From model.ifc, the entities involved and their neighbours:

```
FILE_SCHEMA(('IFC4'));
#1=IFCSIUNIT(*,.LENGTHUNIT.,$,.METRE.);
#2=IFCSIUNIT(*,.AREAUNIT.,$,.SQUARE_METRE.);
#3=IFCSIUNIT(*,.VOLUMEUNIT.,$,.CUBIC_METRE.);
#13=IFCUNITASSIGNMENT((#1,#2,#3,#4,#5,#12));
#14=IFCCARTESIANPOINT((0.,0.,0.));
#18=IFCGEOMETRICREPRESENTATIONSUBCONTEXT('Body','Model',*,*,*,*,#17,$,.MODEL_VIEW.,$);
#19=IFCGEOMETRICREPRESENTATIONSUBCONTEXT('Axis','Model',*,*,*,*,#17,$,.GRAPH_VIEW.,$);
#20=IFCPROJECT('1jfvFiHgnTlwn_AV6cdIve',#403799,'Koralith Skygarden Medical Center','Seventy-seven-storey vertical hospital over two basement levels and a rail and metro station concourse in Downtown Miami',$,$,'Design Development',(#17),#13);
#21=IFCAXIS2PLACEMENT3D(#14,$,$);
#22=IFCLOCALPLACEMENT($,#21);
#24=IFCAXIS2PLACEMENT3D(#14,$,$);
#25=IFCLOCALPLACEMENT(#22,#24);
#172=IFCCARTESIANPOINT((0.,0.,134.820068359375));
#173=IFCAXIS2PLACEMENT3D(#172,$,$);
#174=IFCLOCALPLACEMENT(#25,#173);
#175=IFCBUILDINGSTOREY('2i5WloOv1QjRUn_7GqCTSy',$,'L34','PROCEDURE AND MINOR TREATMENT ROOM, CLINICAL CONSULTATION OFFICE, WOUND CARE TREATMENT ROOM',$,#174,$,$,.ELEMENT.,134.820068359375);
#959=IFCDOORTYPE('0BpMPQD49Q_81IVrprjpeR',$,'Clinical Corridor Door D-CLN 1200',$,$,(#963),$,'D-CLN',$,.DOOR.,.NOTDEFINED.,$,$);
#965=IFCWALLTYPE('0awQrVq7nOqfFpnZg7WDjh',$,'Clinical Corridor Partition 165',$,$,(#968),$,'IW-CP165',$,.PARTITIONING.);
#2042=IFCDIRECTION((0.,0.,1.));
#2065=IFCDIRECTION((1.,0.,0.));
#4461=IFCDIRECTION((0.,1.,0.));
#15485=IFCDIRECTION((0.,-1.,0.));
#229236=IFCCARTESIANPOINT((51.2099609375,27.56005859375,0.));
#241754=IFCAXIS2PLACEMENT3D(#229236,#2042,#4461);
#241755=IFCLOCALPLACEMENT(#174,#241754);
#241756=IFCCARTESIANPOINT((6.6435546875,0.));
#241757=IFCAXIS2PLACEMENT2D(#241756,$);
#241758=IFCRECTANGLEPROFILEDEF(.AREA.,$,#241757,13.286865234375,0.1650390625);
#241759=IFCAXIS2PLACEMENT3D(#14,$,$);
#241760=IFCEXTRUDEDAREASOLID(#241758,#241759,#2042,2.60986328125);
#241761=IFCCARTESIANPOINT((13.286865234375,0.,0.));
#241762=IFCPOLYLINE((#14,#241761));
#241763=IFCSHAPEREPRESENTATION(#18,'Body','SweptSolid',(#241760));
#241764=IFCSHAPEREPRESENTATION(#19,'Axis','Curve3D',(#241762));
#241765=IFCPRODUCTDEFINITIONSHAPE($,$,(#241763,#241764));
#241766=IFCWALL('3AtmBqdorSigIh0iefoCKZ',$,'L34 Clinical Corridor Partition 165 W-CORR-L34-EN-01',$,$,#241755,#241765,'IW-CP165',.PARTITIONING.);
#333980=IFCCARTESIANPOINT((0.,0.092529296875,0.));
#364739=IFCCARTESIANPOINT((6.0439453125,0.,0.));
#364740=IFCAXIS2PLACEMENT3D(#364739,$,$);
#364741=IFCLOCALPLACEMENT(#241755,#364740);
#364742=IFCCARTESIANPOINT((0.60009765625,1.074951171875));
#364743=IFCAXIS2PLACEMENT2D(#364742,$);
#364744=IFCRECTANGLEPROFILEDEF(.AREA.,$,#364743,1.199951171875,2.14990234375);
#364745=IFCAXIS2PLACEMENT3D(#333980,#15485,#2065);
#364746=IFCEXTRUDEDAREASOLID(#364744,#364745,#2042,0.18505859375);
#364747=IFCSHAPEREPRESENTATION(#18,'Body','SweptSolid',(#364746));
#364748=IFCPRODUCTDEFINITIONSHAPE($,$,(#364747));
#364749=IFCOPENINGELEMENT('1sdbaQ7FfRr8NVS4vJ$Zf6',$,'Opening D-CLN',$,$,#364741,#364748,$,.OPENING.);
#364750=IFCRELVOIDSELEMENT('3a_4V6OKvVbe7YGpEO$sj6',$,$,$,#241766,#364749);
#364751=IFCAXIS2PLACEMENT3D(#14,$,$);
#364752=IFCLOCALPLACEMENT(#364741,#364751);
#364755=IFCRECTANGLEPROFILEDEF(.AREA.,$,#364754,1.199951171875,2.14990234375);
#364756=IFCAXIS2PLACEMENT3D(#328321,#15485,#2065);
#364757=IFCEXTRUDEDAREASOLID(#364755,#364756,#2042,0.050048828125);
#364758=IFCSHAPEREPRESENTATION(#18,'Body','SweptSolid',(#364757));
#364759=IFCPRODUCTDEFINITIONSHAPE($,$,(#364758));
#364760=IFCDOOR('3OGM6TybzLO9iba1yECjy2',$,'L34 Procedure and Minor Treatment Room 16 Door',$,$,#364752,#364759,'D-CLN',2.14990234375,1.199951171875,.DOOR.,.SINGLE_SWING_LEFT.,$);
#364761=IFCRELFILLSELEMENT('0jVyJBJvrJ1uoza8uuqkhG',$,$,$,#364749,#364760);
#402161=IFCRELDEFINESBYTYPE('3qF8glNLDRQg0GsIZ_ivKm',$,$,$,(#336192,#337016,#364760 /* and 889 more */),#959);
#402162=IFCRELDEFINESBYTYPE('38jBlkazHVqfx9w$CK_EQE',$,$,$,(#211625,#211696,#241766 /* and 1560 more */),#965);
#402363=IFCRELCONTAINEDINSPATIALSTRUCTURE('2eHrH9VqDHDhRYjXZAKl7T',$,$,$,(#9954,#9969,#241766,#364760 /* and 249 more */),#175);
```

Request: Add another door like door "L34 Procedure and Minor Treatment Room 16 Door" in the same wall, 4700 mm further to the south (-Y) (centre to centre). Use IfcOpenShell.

```python
import ifcopenshell
import ifcopenshell.api.feature
import ifcopenshell.api.geometry
import ifcopenshell.api.root
import ifcopenshell.geom
import ifcopenshell.util.element
import ifcopenshell.util.placement
import ifcopenshell.util.shape
import ifcopenshell.util.unit

model = ifcopenshell.open("model.ifc")
unit_scale = ifcopenshell.util.unit.calculate_unit_scale(model)
settings = ifcopenshell.geom.settings()


def volume(element):
    """Net volume in cubic metres, openings subtracted."""
    shape = ifcopenshell.geom.create_shape(settings, element)
    return ifcopenshell.util.shape.get_volume(shape.geometry)


door = model.by_guid("3OGM6TybzLO9iba1yECjy2")
opening = door.FillsVoids[0].RelatingOpeningElement
wall = opening.VoidsElements[0].RelatingBuildingElement
before = volume(wall)
shift = ifcopenshell.util.placement.get_local_placement(wall.ObjectPlacement)[:3, 0] * -4.7 / unit_scale

# copy_class copies the void relationship, type, container and properties, but no geometry.
new_opening = ifcopenshell.api.root.copy_class(model, product=opening)
new_opening.Representation = ifcopenshell.util.element.copy_deep(
    model, opening.Representation, exclude=["IfcGeometricRepresentationContext", "IfcRepresentationMap"]
)
new_door = ifcopenshell.api.root.copy_class(model, product=door)
new_door.Representation = ifcopenshell.util.element.copy_deep(
    model, door.Representation, exclude=["IfcGeometricRepresentationContext", "IfcRepresentationMap"]
)
new_door.Tag = None
ifcopenshell.api.feature.add_filling(model, opening=new_opening, element=new_door)

for old, new in ((opening, new_opening), (door, new_door)):
    matrix = ifcopenshell.util.placement.get_local_placement(old.ObjectPlacement)
    matrix[:3, 3] += shift
    ifcopenshell.api.geometry.edit_object_placement(model, product=new, matrix=matrix, is_si=False)

after = volume(wall)

print(f"wall volume {before:.3f} -> {after:.3f} m3")

model.write("model_rev.ifc")
```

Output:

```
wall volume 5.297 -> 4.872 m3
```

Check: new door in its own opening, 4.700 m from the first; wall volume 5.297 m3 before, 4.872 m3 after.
